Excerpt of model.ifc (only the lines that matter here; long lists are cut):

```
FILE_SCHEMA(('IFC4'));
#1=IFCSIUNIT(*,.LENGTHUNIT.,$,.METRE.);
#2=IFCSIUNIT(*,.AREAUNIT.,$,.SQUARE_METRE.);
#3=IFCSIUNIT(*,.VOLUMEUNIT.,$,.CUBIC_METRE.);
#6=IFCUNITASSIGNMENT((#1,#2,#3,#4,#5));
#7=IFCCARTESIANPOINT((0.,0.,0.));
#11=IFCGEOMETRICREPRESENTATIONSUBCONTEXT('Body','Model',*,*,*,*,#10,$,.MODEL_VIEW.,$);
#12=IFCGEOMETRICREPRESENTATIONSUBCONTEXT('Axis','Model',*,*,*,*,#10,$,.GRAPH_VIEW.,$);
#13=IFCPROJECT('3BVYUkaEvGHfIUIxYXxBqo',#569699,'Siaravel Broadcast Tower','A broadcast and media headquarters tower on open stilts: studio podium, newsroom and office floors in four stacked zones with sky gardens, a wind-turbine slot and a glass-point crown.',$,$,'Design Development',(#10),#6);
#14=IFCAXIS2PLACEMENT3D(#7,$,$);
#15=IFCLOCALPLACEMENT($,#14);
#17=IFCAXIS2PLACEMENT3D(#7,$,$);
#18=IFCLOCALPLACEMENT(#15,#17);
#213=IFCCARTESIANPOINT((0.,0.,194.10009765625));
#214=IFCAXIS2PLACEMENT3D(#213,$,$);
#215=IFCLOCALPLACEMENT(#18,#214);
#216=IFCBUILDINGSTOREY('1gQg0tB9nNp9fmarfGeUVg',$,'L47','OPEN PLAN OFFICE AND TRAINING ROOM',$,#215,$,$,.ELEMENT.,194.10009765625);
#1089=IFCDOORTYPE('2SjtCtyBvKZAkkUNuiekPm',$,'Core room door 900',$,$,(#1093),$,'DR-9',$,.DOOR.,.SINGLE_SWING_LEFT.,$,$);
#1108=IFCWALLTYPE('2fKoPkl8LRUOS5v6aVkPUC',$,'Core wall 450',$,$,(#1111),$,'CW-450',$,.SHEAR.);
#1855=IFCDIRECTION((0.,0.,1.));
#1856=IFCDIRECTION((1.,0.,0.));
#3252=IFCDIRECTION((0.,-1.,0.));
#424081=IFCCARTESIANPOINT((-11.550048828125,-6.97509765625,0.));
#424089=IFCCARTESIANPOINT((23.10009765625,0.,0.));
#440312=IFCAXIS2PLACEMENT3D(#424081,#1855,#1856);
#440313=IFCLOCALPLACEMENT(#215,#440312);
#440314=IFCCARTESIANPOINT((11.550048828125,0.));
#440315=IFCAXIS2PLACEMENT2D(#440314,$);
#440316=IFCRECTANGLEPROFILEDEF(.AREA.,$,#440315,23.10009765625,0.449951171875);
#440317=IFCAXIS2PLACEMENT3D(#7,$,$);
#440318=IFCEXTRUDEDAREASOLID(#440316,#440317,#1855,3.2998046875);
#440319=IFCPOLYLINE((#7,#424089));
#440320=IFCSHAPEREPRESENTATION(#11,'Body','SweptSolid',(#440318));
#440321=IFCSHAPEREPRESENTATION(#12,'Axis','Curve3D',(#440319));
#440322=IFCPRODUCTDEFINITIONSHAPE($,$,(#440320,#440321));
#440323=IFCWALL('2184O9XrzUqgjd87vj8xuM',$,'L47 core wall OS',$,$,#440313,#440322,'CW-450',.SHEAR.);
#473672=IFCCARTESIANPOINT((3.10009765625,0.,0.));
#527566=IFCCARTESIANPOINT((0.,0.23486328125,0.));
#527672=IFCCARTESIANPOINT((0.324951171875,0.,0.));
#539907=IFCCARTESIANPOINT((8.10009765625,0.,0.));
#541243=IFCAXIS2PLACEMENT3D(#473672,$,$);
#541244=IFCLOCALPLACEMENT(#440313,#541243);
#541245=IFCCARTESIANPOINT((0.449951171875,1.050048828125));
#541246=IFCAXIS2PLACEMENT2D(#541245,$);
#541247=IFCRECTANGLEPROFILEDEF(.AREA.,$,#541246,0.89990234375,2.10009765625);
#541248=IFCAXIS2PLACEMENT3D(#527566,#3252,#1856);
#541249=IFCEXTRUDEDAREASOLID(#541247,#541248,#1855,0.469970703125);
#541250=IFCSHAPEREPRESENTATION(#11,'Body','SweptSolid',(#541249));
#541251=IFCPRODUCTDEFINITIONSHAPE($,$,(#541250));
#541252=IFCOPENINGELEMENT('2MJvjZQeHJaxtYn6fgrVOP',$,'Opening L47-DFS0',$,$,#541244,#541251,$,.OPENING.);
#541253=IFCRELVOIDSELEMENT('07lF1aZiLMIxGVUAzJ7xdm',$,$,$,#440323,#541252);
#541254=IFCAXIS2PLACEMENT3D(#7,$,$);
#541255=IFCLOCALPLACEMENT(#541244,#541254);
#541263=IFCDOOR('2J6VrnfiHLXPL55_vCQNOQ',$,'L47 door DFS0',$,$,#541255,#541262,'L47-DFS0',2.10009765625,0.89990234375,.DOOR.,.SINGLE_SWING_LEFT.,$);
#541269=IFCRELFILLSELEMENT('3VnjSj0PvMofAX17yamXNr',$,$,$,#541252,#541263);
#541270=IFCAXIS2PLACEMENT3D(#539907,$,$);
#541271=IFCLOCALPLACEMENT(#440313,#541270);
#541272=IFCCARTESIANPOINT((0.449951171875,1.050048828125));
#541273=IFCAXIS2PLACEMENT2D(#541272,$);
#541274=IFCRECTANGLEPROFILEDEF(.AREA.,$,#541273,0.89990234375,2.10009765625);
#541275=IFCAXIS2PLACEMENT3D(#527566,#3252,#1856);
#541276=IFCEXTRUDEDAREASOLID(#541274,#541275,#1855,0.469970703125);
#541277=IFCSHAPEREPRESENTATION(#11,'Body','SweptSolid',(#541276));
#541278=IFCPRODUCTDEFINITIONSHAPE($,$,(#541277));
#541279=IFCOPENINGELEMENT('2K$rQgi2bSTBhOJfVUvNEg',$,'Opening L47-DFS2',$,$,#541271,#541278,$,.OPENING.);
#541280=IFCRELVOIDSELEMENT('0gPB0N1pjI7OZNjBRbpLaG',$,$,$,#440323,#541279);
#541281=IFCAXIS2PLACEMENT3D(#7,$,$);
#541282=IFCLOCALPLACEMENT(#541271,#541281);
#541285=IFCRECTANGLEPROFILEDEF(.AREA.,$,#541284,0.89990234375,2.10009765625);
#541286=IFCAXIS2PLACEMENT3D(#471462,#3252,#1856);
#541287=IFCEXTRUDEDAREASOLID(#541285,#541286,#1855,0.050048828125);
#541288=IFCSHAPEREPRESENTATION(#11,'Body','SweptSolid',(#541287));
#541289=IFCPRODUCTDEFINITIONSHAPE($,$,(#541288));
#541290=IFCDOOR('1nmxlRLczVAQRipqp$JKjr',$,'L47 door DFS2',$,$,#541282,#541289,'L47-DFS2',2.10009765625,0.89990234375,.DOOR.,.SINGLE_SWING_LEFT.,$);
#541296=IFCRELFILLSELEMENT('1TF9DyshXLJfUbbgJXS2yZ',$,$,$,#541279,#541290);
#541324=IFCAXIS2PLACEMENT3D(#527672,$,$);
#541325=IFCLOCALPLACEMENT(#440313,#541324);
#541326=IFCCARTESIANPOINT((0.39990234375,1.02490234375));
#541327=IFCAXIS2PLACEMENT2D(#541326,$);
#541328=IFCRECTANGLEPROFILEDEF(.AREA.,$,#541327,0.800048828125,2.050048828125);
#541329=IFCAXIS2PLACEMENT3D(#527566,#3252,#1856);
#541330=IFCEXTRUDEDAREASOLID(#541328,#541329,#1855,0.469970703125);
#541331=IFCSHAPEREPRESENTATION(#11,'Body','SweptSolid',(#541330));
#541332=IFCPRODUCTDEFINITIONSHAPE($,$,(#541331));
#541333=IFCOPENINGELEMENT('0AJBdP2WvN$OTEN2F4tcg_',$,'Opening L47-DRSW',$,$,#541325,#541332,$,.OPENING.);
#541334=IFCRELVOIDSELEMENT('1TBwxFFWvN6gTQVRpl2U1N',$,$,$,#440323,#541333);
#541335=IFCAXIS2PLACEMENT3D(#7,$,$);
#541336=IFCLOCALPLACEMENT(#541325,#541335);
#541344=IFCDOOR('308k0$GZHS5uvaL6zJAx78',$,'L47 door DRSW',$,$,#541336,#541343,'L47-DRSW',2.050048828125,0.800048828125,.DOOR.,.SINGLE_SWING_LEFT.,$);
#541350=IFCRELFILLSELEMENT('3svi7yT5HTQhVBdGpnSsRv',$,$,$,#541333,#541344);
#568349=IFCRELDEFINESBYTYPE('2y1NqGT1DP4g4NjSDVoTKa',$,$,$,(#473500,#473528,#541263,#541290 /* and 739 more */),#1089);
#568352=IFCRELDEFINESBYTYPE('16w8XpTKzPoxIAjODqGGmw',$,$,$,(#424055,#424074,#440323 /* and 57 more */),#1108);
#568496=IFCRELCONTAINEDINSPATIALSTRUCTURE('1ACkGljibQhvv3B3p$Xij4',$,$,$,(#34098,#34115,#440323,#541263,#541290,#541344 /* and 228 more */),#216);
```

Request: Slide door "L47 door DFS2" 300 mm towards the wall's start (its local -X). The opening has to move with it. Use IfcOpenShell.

```python
import ifcopenshell
import ifcopenshell.api.geometry
import ifcopenshell.util.placement
import ifcopenshell.util.unit

model = ifcopenshell.open("model.ifc")
unit_scale = ifcopenshell.util.unit.calculate_unit_scale(model)

door = model.by_id(541290)
opening = door.FillsVoids[0].RelatingOpeningElement
wall = opening.VoidsElements[0].RelatingBuildingElement

wall_matrix = ifcopenshell.util.placement.get_local_placement(wall.ObjectPlacement)
shift = wall_matrix[:3, 0] * -0.3 / unit_scale
before = ifcopenshell.util.placement.get_local_placement(door.ObjectPlacement)[:3, 3].copy()

# The door is placed relative to its opening, so it follows when the opening moves.
matrix = ifcopenshell.util.placement.get_local_placement(opening.ObjectPlacement)
matrix[:3, 3] += shift
ifcopenshell.api.geometry.edit_object_placement(
    model, product=opening, matrix=matrix, is_si=False, should_transform_children=True
)

after = ifcopenshell.util.placement.get_local_placement(door.ObjectPlacement)[:3, 3]
print("door moved by", (after - before).round(3) + 0.0)

model.write("model_rev.ifc")
```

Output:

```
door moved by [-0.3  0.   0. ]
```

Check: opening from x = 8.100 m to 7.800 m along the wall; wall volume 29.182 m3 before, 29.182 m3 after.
